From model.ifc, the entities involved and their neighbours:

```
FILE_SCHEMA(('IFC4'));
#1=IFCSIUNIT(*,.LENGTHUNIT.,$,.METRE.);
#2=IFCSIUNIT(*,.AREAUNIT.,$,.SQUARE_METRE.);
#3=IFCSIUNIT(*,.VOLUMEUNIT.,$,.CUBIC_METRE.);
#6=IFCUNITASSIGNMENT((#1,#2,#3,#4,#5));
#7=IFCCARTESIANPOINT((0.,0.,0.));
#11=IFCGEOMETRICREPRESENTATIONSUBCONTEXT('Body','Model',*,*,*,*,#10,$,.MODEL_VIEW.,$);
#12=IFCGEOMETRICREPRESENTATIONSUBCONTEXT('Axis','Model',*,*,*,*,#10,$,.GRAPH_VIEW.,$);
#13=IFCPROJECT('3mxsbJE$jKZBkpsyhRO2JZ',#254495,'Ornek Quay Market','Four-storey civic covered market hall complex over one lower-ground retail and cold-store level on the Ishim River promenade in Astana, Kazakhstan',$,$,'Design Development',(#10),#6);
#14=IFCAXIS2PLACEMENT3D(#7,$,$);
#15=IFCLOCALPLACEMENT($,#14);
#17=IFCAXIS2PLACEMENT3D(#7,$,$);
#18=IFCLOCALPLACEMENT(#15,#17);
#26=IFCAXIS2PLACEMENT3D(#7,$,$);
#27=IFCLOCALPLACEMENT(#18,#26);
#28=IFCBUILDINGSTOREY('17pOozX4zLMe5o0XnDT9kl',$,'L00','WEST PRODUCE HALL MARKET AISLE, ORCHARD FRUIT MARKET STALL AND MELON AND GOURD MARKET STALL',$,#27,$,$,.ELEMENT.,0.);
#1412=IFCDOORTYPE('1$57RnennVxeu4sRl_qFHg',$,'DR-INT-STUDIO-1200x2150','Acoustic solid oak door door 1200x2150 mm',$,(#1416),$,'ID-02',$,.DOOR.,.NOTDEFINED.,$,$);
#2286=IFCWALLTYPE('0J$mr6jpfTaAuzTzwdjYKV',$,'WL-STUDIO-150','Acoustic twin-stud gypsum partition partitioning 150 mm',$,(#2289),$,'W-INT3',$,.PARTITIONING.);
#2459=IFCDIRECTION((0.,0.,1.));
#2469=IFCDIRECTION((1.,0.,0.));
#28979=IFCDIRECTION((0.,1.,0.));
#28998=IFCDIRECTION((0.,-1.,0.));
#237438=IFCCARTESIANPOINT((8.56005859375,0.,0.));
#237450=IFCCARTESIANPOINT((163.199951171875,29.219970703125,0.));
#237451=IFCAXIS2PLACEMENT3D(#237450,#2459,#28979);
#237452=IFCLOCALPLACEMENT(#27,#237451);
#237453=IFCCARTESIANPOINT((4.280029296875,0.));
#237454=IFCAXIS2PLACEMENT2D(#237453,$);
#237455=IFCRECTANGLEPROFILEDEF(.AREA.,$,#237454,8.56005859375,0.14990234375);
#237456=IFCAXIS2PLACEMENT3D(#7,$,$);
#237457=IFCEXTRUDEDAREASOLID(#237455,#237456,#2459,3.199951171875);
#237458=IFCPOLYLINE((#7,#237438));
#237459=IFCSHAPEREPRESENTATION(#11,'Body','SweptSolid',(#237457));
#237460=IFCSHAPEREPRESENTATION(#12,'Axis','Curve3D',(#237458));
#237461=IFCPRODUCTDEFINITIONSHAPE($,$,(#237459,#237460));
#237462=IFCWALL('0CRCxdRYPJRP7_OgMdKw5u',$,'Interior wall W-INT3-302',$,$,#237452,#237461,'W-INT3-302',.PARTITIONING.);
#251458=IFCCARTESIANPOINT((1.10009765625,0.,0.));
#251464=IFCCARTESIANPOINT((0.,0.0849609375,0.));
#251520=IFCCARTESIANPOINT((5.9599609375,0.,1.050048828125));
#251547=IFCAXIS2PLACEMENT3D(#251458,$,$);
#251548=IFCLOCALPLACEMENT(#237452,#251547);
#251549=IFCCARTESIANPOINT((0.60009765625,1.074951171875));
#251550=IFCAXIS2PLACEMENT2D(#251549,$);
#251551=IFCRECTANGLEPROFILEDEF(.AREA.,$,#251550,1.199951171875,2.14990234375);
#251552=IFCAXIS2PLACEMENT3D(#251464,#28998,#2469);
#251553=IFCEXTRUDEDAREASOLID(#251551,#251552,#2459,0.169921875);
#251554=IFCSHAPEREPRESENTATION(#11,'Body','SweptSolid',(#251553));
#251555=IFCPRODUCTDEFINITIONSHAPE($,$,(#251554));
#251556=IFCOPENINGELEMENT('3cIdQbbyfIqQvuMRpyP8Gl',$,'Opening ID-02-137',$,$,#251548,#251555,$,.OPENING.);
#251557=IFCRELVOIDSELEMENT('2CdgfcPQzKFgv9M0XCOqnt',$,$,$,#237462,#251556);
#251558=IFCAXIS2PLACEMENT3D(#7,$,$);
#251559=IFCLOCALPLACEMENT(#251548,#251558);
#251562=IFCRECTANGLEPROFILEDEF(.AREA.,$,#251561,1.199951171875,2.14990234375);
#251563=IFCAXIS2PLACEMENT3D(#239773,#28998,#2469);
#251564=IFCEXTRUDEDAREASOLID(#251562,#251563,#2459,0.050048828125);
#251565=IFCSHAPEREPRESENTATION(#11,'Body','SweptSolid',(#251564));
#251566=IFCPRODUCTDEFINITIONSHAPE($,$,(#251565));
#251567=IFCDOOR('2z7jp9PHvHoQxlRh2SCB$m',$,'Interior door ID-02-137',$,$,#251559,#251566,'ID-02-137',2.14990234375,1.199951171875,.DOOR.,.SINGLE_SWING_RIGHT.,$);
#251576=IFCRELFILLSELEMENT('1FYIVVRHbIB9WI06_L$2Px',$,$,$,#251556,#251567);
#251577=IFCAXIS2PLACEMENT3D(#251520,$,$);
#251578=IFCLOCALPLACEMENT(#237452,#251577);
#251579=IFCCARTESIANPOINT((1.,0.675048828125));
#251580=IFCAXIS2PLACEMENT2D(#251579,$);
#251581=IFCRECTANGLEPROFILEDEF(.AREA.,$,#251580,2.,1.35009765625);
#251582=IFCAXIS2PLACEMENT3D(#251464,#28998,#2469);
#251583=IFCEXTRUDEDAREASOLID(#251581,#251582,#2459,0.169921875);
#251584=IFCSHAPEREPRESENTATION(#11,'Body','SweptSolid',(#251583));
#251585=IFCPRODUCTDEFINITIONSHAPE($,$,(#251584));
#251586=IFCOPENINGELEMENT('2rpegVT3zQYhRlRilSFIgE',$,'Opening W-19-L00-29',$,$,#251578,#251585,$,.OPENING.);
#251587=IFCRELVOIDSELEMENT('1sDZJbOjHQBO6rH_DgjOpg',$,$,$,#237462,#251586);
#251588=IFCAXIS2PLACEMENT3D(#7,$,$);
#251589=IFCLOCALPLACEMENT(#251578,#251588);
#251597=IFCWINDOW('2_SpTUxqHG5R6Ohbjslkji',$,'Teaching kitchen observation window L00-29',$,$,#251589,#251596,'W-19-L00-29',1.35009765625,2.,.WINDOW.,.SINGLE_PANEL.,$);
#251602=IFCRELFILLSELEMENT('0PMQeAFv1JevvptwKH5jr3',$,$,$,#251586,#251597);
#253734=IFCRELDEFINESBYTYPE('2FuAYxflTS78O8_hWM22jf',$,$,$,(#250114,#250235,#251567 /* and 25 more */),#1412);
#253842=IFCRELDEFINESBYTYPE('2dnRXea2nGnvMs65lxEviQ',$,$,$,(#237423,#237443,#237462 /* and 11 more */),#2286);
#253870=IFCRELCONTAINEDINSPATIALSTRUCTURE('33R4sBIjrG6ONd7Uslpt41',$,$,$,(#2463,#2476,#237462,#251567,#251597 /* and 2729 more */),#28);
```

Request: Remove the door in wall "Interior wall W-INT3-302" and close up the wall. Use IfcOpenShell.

```python
import ifcopenshell
import ifcopenshell.api.feature
import ifcopenshell.api.root
import ifcopenshell.geom
import ifcopenshell.util.shape

model = ifcopenshell.open("model.ifc")
settings = ifcopenshell.geom.settings()


def volume(element):
    """Net volume in cubic metres, openings subtracted."""
    shape = ifcopenshell.geom.create_shape(settings, element)
    return ifcopenshell.util.shape.get_volume(shape.geometry)


door = model.by_guid("2z7jp9PHvHoQxlRh2SCB$m")
opening = door.FillsVoids[0].RelatingOpeningElement
wall = opening.VoidsElements[0].RelatingBuildingElement
before = volume(wall)

ifcopenshell.api.root.remove_product(model, product=door)
ifcopenshell.api.feature.remove_feature(model, feature=opening)

after = volume(wall)

print(f"wall volume {before:.3f} -> {after:.3f} m3")

model.write("model_updated.ifc")
```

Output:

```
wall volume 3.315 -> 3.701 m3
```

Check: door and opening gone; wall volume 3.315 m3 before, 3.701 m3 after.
